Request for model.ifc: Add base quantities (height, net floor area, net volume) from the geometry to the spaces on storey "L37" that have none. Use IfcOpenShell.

First a look at what the model holds.

```python
import ifcopenshell
import ifcopenshell.util.element
import ifcopenshell.util.unit

model = ifcopenshell.open("model.ifc")
print(model.schema)
for unit_type in ("LENGTHUNIT", "AREAUNIT", "VOLUMEUNIT"):
    print(unit_type, ifcopenshell.util.unit.calculate_unit_scale(model, unit_type))
storey = next(s for s in model.by_type("IfcBuildingStorey") if s.Name == "L37")
spaces = [e for e in ifcopenshell.util.element.get_decomposition(storey) if e.is_a("IfcSpace")]
for e in sorted(spaces, key=lambda e: e.id()):
    print(e.id(), e.is_a(), e.Name, list(ifcopenshell.util.element.get_psets(e, qtos_only=True)), sep=" | ")
```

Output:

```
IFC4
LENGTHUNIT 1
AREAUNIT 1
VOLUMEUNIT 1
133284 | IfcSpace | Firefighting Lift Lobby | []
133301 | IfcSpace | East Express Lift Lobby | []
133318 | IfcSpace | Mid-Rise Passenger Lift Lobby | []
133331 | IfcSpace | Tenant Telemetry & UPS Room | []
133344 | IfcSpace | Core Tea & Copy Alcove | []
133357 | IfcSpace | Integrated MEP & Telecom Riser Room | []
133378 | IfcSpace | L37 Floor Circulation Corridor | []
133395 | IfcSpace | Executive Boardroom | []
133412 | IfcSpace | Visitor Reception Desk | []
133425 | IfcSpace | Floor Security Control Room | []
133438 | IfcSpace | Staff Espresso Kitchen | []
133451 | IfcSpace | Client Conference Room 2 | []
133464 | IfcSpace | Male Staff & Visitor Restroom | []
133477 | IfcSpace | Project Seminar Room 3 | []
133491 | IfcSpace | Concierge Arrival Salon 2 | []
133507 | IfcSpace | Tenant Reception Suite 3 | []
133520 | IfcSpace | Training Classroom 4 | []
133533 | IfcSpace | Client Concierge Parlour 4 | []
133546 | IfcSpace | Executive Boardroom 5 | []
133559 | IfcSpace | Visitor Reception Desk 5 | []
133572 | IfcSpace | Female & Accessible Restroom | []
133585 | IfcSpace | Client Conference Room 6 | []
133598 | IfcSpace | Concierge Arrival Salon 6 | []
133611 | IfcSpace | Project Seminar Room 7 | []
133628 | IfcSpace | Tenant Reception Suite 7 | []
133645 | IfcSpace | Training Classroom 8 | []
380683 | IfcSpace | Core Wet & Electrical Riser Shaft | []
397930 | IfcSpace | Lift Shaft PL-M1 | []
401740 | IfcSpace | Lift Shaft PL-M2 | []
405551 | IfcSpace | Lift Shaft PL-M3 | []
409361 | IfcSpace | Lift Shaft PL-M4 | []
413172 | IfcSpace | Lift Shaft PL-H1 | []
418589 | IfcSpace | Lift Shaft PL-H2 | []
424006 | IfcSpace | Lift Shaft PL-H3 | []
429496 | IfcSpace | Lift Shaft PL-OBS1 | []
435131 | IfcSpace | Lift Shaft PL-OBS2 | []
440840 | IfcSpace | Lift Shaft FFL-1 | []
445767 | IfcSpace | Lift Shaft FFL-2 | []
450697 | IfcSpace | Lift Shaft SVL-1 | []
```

```python
import ifcopenshell
import ifcopenshell.api.pset
import ifcopenshell.geom
import ifcopenshell.util.element
import ifcopenshell.util.shape
import ifcopenshell.util.unit

model = ifcopenshell.open("model.ifc")
unit_scale = ifcopenshell.util.unit.calculate_unit_scale(model)
area_scale = ifcopenshell.util.unit.calculate_unit_scale(model, "AREAUNIT")
volume_scale = ifcopenshell.util.unit.calculate_unit_scale(model, "VOLUMEUNIT")
settings = ifcopenshell.geom.settings()

storey = next(s for s in model.by_type("IfcBuildingStorey") if s.Name == "L37")
spaces = [e for e in ifcopenshell.util.element.get_decomposition(storey) if e.is_a("IfcSpace")]

for e in sorted(spaces, key=lambda e: e.id()):
    if ifcopenshell.util.element.get_psets(e, qtos_only=True, should_inherit=False):
        continue
    # Geometry comes back in metres, in the element's own axes.
    shape = ifcopenshell.geom.create_shape(settings, e)
    values = {
        "Height": ifcopenshell.util.shape.get_z(shape.geometry) / unit_scale,
        "NetFloorArea": ifcopenshell.util.shape.get_footprint_area(shape.geometry) / area_scale,
        "NetVolume": ifcopenshell.util.shape.get_volume(shape.geometry) / volume_scale,
    }
    qto = ifcopenshell.api.pset.add_qto(model, product=e, name="Qto_SpaceBaseQuantities")
    ifcopenshell.api.pset.edit_qto(model, qto=qto, properties=values)
    print(e.id(), {k: round(v, 3) for k, v in values.items()})

model.write("model_rev.ifc")
```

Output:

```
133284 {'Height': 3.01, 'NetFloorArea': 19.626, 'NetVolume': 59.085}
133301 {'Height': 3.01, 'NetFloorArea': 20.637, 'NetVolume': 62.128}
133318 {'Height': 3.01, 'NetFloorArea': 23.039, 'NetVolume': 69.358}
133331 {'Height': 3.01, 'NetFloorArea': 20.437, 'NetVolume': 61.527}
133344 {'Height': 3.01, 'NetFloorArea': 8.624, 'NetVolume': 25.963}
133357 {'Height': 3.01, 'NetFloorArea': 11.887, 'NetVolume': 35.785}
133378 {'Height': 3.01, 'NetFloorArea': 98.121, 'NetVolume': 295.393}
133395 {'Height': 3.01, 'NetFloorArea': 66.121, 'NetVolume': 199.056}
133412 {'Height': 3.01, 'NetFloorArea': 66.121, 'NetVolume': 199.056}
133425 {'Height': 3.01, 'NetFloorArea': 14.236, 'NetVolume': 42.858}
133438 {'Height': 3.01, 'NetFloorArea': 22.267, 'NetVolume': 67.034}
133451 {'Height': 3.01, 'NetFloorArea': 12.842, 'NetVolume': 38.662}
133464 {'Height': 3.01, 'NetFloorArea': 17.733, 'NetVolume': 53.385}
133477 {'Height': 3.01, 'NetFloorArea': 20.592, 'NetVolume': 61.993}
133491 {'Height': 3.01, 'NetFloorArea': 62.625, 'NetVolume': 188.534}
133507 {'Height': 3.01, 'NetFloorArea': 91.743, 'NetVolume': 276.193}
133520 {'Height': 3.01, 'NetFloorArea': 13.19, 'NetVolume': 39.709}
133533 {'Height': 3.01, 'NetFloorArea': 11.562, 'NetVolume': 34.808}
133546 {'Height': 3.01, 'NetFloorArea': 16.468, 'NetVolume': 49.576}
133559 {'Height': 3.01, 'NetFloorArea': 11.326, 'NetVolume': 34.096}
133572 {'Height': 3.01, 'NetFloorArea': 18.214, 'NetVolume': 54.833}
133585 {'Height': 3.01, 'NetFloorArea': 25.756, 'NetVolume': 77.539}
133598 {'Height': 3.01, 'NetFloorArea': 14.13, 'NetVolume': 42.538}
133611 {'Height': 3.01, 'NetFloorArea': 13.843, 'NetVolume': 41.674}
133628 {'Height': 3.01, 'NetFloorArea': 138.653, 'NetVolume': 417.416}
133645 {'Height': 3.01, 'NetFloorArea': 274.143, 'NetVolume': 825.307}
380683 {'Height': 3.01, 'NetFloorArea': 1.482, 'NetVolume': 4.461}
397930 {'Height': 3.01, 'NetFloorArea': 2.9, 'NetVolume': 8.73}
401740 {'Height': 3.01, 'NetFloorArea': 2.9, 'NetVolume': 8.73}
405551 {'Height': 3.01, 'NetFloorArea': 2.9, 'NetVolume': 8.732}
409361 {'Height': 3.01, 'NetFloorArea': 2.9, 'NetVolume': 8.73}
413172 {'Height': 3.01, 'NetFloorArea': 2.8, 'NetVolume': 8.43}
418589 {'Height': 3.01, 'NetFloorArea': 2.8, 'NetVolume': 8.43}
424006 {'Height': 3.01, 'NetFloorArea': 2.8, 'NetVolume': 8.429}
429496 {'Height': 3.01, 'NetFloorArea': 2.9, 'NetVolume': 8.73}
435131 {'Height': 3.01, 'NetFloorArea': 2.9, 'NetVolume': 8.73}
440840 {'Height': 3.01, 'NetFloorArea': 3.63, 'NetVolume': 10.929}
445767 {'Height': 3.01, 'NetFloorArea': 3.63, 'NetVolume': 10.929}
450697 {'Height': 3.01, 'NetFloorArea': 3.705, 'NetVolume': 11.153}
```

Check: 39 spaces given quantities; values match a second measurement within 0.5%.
